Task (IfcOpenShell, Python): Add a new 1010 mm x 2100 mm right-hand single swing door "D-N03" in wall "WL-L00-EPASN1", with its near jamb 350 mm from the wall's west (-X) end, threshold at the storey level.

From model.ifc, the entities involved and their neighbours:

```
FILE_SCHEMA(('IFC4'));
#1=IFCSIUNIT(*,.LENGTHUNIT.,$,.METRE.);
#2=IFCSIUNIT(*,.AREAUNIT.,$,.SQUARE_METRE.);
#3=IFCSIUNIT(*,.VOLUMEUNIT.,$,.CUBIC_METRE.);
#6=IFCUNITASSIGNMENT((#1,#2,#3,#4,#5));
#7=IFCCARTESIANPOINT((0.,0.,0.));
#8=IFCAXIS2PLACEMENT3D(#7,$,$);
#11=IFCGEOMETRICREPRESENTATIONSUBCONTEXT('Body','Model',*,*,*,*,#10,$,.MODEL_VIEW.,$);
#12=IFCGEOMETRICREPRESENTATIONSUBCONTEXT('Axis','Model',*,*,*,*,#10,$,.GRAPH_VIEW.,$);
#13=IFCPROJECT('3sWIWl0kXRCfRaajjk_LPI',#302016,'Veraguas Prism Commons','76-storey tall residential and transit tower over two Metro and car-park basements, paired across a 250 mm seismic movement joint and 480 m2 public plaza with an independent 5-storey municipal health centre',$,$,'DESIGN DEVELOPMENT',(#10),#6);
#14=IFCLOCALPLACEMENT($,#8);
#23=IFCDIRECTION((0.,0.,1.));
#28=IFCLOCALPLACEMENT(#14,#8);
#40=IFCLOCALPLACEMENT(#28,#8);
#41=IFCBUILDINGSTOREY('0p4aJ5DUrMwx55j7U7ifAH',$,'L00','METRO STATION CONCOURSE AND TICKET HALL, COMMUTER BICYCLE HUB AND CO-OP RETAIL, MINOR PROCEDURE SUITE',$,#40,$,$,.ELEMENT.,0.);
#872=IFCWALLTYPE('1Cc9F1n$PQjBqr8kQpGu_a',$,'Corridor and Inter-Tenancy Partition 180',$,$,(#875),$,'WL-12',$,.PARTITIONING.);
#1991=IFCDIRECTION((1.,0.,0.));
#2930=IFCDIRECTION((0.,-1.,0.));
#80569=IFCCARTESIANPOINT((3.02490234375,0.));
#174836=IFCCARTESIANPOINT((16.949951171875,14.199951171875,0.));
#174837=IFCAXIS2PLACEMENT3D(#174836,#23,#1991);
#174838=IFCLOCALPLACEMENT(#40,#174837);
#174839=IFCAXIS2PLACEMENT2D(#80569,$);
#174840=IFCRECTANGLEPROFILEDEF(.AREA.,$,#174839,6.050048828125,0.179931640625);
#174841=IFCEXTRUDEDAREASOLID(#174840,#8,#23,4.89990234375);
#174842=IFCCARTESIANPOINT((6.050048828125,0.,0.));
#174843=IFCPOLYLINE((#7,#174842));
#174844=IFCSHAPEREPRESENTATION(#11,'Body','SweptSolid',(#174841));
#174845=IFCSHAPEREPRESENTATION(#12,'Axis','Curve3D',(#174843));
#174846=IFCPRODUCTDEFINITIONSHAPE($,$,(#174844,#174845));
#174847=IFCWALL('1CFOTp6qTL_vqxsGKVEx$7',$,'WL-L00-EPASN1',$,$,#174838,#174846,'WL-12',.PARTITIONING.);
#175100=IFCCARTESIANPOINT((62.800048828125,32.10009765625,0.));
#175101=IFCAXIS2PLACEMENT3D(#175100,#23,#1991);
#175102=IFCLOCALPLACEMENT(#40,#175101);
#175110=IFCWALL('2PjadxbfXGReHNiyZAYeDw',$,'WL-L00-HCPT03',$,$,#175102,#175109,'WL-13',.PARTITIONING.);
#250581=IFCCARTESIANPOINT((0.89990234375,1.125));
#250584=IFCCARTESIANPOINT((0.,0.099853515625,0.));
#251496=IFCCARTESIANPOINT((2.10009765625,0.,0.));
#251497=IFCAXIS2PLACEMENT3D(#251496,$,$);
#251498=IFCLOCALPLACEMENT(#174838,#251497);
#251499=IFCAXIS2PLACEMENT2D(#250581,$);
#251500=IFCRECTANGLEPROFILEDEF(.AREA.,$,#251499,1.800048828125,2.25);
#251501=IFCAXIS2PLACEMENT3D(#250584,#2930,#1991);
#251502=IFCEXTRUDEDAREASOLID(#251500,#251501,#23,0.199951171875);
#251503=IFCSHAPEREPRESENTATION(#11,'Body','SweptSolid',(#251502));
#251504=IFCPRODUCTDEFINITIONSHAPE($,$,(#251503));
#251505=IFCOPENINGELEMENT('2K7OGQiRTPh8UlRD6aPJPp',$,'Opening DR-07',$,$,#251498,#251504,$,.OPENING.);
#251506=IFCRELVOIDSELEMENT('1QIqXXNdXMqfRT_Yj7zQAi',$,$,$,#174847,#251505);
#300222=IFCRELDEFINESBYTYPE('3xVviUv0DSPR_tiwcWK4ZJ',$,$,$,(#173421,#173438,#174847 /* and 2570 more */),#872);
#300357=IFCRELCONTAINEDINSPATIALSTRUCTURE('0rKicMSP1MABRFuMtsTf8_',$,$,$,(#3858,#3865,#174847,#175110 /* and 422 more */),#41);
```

```python
import numpy as np
import ifcopenshell
import ifcopenshell.api.feature
import ifcopenshell.api.geometry
import ifcopenshell.api.root
import ifcopenshell.api.spatial
import ifcopenshell.geom
import ifcopenshell.util.element
import ifcopenshell.util.placement
import ifcopenshell.util.representation
import ifcopenshell.util.shape
import ifcopenshell.util.unit

model = ifcopenshell.open("model.ifc")
unit_scale = ifcopenshell.util.unit.calculate_unit_scale(model)
settings = ifcopenshell.geom.settings()


def volume(element):
    """Net volume in cubic metres, openings subtracted."""
    shape = ifcopenshell.geom.create_shape(settings, element)
    return ifcopenshell.util.shape.get_volume(shape.geometry)


wall = model.by_id(174847)
storey = ifcopenshell.util.element.get_container(wall, ifc_class="IfcBuildingStorey")
context = ifcopenshell.util.representation.get_context(model, "Model", "Body", "MODEL_VIEW")
before = volume(wall)

width, height, from_end, sill = 1.01, 2.1, 0.35, 0.0  # metres

# The wall runs along its own X axis, and the end named is its -X end.
wall_shape = ifcopenshell.geom.create_shape(settings, wall)
x, y, z = ifcopenshell.util.shape.get_vertices(wall_shape.geometry).T
start = x.min() + from_end
face, thickness = float(y.min()), float(y.max() - y.min())
wall_matrix = ifcopenshell.util.placement.get_local_placement(wall.ObjectPlacement)
level = ifcopenshell.util.placement.get_local_placement(storey.ObjectPlacement)[2, 3]


def in_wall(x, y):
    """Placement at x, y metres in the wall's axes, at sill height."""
    matrix = wall_matrix.copy()
    matrix[:, 3] = wall_matrix @ np.array([x / unit_scale, y / unit_scale, 0.0, 1.0])
    matrix[2, 3] = level + sill / unit_scale
    return matrix


# Opening: a box that overshoots both wall faces by 50 mm.
opening = ifcopenshell.api.root.create_entity(model, ifc_class="IfcOpeningElement", predefined_type="OPENING")
box = ifcopenshell.api.geometry.add_wall_representation(
    model, context=context, length=width, height=height, thickness=thickness + 0.1
)
ifcopenshell.api.geometry.assign_representation(model, product=opening, representation=box)
ifcopenshell.api.geometry.edit_object_placement(model, product=opening, matrix=in_wall(start, face - 0.05), is_si=False)
ifcopenshell.api.feature.add_feature(model, feature=opening, element=wall)

door = ifcopenshell.api.root.create_entity(model, ifc_class="IfcDoor", name="D-N03", predefined_type="DOOR")
door.OverallWidth, door.OverallHeight = width / unit_scale, height / unit_scale
door.OperationType = "SINGLE_SWING_RIGHT"
body = ifcopenshell.api.geometry.add_door_representation(
    model,
    context=context,
    overall_width=door.OverallWidth,
    overall_height=door.OverallHeight,
    operation_type="SINGLE_SWING_RIGHT",
    lining_properties={"LiningDepth": thickness / unit_scale, "ThresholdDepth": thickness / unit_scale},
)
ifcopenshell.api.geometry.assign_representation(model, product=door, representation=body)
ifcopenshell.api.spatial.assign_container(model, products=[door], relating_structure=storey)
ifcopenshell.api.feature.add_filling(model, opening=opening, element=door)

# The lining spans the wall, so the door starts at the wall face.
ifcopenshell.api.geometry.edit_object_placement(model, product=door, matrix=in_wall(start, face), is_si=False)

after = volume(wall)

print(f"wall volume {before:.3f} -> {after:.3f} m3")

model.write("model_rev.ifc")
```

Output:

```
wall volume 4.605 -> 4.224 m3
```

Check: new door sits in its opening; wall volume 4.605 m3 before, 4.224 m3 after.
